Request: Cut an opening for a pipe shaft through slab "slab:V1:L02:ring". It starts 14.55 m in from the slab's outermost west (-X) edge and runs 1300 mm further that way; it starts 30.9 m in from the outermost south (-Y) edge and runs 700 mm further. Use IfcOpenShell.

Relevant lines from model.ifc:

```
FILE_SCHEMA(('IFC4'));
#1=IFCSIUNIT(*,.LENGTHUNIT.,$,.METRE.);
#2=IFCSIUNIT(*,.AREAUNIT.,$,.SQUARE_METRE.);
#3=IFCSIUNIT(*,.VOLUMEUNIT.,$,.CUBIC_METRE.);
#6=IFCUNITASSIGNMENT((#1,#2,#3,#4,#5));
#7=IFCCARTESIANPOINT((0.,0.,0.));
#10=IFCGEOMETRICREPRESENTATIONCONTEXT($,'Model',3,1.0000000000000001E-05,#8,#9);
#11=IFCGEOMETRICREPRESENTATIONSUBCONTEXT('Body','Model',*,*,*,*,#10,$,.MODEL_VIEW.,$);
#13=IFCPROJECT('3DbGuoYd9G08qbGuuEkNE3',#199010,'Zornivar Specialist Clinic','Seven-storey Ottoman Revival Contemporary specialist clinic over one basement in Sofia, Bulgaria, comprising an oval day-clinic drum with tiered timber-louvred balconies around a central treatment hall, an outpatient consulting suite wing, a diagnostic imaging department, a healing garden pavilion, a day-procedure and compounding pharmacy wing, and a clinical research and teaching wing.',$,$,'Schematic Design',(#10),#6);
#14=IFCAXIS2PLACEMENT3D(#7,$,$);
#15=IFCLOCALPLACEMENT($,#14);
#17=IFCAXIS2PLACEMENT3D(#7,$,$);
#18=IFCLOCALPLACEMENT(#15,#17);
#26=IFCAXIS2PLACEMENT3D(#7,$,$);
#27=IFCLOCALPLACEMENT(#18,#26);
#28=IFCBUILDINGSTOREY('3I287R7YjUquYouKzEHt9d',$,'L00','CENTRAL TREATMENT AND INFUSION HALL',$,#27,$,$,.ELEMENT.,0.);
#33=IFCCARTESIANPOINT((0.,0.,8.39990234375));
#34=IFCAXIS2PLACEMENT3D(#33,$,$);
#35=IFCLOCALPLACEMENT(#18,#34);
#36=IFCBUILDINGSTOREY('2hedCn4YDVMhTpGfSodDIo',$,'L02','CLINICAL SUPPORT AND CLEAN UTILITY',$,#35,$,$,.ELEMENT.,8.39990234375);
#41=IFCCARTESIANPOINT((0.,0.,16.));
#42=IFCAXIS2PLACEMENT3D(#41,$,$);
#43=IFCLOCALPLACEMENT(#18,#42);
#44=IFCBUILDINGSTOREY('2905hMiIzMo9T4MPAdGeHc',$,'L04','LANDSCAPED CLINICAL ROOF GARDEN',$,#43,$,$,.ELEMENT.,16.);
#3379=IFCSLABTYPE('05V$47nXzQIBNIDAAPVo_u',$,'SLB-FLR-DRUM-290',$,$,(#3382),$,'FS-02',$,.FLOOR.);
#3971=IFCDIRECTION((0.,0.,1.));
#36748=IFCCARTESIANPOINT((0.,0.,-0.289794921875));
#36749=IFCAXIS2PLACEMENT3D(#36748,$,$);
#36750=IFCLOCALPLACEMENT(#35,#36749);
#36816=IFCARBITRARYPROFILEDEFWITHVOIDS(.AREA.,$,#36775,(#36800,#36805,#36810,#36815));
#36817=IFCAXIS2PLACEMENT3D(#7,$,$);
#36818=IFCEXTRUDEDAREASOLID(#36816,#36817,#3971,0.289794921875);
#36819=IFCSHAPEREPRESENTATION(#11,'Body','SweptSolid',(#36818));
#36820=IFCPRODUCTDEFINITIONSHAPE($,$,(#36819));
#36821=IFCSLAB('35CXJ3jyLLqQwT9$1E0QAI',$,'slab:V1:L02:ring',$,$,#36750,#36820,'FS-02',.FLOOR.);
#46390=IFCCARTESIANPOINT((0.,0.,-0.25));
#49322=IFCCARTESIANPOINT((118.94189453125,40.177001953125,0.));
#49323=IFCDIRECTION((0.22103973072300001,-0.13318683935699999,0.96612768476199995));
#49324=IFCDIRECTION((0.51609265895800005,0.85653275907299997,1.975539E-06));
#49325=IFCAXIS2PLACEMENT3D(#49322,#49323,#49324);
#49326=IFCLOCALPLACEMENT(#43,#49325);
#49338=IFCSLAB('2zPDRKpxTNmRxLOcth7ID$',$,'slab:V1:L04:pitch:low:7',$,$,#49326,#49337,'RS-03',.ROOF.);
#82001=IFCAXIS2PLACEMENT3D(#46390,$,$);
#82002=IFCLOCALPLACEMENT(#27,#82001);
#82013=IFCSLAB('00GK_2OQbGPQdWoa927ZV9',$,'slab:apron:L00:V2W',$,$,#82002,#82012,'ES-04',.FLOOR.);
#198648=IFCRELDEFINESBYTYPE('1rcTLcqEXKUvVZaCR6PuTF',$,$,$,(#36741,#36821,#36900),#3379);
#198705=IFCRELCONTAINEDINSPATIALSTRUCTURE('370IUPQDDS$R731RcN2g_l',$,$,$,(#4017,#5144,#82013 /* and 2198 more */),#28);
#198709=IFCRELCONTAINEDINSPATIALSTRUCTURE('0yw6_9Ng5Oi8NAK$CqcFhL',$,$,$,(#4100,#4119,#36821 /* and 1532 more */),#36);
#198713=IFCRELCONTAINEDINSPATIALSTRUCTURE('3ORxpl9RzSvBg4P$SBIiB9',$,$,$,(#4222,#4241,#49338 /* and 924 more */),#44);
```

```python
import numpy as np
import ifcopenshell
import ifcopenshell.api.feature
import ifcopenshell.api.geometry
import ifcopenshell.api.root
import ifcopenshell.geom
import ifcopenshell.util.placement
import ifcopenshell.util.representation
import ifcopenshell.util.shape
import ifcopenshell.util.unit

model = ifcopenshell.open("model.ifc")
unit_scale = ifcopenshell.util.unit.calculate_unit_scale(model)
settings = ifcopenshell.geom.settings()


def volume(element):
    """Net volume in cubic metres, openings subtracted."""
    shape = ifcopenshell.geom.create_shape(settings, element)
    return ifcopenshell.util.shape.get_volume(shape.geometry)


slab = model.by_id(36821)
before = volume(slab)

# Extent in the slab's own axes, in metres. The edges named are its -X and -Y sides.
slab_shape = ifcopenshell.geom.create_shape(settings, slab)
vertices = ifcopenshell.util.shape.get_vertices(slab_shape.geometry)
x_min, y_min, bottom = vertices.min(axis=0)
top = vertices[:, 2].max()

opening = ifcopenshell.api.root.create_entity(model, ifc_class="IfcOpeningElement", name="Pipe shaft opening", predefined_type="OPENING")
context = ifcopenshell.util.representation.get_context(model, "Model", "Body", "MODEL_VIEW")
width, depth = 1.3, 0.7
outline = [(0.0, 0.0), (width, 0.0), (width, depth), (0.0, depth), (0.0, 0.0)]
# Overshoot both faces by 50 mm so the cut is clean.
shape = ifcopenshell.api.geometry.add_slab_representation(
    model, context=context, depth=top - bottom + 0.1, polyline=outline
)
ifcopenshell.api.geometry.assign_representation(model, product=opening, representation=shape)

matrix = ifcopenshell.util.placement.get_local_placement(slab.ObjectPlacement)
matrix[:, 3] = matrix @ np.append(np.array([x_min + 14.55, y_min + 30.9, bottom - 0.05]) / unit_scale, 1.0)
ifcopenshell.api.geometry.edit_object_placement(model, product=opening, matrix=matrix, is_si=False)
ifcopenshell.api.feature.add_feature(model, feature=opening, element=slab)

after = volume(slab)

print(f"slab volume {before:.3f} -> {after:.3f} m3")

model.write("model_v2.ifc")
```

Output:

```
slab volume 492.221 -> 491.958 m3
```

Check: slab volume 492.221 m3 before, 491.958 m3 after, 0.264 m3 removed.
